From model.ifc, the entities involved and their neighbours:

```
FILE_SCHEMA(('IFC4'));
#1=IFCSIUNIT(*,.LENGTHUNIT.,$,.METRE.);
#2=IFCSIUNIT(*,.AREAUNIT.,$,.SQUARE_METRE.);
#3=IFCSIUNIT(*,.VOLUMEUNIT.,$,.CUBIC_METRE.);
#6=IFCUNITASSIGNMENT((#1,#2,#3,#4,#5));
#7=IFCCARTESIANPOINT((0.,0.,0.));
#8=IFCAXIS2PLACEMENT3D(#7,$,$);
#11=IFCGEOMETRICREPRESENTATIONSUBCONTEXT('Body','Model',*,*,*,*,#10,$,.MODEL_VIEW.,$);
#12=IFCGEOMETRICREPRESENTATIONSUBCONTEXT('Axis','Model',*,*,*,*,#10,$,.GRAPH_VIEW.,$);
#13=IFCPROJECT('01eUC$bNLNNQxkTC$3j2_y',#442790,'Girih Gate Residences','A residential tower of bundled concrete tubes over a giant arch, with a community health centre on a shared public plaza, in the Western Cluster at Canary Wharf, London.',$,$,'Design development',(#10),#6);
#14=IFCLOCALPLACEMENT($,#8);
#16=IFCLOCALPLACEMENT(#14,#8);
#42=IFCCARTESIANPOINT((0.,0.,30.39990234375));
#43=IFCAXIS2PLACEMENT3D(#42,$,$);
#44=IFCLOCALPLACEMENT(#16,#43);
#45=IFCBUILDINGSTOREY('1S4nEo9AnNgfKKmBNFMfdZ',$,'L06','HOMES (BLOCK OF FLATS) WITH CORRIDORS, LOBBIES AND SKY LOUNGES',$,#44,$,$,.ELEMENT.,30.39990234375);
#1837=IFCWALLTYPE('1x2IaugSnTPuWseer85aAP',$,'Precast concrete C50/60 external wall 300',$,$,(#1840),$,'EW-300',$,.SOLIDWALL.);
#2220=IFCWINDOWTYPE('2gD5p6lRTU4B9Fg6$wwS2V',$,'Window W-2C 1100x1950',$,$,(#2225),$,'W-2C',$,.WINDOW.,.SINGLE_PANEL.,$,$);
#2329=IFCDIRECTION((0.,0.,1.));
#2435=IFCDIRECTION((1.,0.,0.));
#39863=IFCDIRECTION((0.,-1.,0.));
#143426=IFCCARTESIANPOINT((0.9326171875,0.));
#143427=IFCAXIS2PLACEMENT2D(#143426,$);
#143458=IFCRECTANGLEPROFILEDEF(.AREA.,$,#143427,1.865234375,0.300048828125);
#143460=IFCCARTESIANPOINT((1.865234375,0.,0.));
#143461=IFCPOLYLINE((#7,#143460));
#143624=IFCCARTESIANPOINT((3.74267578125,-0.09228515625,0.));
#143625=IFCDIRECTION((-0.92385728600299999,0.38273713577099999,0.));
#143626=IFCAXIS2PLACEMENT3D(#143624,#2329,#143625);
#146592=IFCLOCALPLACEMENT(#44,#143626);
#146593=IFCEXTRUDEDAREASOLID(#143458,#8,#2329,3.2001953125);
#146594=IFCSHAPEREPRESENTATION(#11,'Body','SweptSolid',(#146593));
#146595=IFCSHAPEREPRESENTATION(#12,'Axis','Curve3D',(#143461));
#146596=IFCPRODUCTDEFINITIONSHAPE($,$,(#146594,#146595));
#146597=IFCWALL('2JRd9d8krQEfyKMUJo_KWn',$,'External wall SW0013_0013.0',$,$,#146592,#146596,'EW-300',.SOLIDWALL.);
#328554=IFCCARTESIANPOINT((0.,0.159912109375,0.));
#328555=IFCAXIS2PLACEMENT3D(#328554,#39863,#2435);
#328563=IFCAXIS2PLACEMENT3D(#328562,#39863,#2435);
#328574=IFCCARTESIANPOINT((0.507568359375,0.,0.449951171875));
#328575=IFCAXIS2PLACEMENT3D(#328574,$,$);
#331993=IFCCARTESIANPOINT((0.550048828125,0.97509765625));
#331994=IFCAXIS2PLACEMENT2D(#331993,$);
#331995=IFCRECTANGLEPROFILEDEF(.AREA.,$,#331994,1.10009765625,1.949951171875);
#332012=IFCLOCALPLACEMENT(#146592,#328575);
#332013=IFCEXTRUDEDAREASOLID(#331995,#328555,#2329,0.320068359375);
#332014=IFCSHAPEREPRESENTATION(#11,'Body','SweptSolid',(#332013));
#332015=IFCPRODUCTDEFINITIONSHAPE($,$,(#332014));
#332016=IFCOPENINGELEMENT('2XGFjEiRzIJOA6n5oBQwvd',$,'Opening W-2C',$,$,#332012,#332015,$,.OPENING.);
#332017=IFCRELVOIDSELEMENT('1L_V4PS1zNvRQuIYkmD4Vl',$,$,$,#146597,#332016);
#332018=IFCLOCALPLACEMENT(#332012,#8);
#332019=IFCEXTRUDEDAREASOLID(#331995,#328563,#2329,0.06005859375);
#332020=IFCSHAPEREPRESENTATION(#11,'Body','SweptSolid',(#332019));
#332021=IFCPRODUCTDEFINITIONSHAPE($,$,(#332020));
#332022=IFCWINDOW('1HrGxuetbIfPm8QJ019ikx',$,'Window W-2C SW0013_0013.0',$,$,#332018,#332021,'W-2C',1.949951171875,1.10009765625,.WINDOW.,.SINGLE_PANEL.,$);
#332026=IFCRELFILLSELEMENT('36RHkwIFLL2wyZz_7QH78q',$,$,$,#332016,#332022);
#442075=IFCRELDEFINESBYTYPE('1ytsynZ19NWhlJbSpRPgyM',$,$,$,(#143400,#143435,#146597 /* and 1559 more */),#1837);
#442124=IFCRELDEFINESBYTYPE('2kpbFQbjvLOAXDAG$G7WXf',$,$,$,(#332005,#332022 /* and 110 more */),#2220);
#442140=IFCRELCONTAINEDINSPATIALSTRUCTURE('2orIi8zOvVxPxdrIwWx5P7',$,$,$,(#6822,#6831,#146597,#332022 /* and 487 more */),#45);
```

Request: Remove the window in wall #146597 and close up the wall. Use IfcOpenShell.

```python
import ifcopenshell
import ifcopenshell.api.feature
import ifcopenshell.api.root
import ifcopenshell.geom
import ifcopenshell.util.shape

model = ifcopenshell.open("model.ifc")
settings = ifcopenshell.geom.settings()


def volume(element):
    """Net volume in cubic metres, openings subtracted."""
    shape = ifcopenshell.geom.create_shape(settings, element)
    return ifcopenshell.util.shape.get_volume(shape.geometry)


window = model.by_guid("1HrGxuetbIfPm8QJ019ikx")
opening = window.FillsVoids[0].RelatingOpeningElement
wall = opening.VoidsElements[0].RelatingBuildingElement
before = volume(wall)

ifcopenshell.api.root.remove_product(model, product=window)
ifcopenshell.api.feature.remove_feature(model, feature=opening)

after = volume(wall)

print(f"wall volume {before:.3f} -> {after:.3f} m3")

model.write("model_updated.ifc")
```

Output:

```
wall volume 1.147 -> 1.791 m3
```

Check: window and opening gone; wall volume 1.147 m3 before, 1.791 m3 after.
